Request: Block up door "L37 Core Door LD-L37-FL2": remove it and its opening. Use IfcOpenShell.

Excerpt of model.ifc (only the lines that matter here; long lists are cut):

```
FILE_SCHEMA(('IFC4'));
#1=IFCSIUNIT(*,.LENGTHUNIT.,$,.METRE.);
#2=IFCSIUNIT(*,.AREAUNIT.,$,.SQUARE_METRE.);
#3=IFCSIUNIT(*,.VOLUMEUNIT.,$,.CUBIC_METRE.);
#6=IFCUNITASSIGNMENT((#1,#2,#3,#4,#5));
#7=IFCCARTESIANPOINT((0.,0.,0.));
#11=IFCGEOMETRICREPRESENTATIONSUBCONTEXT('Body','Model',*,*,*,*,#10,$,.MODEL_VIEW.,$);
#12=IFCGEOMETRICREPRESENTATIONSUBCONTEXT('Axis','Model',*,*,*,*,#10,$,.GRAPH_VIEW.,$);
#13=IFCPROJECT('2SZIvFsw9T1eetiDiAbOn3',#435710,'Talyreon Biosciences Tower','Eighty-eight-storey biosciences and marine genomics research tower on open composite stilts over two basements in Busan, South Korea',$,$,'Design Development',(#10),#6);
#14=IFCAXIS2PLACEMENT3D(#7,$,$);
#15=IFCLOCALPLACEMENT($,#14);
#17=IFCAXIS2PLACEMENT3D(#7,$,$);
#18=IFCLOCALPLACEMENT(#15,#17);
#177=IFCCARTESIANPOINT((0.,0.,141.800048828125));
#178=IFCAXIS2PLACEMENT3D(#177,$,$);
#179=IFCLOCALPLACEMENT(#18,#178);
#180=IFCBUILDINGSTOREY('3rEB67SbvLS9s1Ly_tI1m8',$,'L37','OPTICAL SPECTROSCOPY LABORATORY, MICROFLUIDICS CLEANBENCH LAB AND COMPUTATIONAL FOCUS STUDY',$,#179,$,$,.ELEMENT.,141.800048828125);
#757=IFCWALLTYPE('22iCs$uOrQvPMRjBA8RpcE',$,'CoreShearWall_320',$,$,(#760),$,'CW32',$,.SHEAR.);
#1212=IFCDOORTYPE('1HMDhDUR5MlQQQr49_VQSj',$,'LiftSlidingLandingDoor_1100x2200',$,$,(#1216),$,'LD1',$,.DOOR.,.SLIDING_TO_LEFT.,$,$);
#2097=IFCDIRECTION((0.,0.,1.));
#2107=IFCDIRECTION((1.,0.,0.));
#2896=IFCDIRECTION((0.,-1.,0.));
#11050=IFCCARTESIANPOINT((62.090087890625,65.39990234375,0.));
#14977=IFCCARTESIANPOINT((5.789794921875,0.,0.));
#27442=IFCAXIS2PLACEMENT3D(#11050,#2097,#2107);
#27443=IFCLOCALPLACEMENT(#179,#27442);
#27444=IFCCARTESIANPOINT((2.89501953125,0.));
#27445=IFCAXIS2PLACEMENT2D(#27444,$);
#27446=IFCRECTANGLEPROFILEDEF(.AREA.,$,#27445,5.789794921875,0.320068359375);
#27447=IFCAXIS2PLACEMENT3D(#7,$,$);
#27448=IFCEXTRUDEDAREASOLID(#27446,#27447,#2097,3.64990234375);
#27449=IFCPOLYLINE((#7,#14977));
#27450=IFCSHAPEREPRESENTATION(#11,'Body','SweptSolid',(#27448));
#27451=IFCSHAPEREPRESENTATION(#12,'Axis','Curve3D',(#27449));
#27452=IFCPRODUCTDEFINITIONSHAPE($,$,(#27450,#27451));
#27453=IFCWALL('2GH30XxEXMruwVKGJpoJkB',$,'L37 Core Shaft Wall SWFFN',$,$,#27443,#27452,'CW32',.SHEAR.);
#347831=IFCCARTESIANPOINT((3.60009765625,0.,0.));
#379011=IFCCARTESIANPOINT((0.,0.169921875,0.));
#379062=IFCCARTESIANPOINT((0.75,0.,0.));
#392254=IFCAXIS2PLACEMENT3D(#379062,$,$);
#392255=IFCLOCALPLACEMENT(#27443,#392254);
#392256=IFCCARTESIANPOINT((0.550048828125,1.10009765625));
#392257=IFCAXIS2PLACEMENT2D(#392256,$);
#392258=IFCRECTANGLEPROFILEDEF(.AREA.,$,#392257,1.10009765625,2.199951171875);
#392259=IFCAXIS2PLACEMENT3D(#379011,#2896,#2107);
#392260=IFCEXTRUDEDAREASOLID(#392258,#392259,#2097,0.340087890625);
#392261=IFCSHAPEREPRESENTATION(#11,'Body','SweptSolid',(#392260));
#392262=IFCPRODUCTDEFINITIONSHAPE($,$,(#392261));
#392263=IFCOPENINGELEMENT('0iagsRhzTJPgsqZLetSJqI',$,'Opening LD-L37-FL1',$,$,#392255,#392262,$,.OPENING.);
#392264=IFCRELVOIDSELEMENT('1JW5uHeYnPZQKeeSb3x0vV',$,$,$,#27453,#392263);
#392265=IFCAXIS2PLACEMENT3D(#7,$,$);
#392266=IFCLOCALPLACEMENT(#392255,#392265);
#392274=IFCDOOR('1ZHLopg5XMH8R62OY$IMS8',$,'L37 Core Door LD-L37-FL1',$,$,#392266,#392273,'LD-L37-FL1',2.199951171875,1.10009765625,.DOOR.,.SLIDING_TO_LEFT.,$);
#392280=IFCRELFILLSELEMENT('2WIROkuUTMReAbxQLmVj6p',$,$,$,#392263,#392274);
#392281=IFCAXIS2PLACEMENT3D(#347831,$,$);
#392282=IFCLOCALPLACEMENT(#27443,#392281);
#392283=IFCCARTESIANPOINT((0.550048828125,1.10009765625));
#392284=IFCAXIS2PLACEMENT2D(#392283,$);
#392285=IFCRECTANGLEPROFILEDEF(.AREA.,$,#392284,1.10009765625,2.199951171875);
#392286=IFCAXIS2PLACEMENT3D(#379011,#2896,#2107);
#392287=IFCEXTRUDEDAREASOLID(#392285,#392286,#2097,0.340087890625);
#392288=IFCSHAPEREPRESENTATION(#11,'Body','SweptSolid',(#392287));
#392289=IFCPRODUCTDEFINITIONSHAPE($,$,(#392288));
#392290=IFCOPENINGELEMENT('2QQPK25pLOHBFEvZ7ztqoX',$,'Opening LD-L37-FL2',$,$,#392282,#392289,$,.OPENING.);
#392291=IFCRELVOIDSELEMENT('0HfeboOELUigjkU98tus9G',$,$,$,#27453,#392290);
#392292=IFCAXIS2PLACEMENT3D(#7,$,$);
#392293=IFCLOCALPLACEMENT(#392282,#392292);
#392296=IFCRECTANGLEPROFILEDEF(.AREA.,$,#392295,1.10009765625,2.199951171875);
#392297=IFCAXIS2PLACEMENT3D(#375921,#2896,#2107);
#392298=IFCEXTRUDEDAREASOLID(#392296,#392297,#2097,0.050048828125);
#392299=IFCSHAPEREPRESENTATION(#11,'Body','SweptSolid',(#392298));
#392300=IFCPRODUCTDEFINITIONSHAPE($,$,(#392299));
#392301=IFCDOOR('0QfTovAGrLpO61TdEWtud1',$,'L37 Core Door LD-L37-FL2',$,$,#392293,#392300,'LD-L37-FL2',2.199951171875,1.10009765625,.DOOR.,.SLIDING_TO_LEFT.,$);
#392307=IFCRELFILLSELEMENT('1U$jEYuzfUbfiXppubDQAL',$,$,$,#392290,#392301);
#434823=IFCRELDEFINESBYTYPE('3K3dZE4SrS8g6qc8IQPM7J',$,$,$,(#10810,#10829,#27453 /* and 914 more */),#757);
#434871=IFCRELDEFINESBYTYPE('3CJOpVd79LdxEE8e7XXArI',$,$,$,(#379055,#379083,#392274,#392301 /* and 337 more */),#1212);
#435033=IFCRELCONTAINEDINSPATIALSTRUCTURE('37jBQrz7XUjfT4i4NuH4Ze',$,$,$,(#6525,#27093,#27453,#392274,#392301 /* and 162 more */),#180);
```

```python
import ifcopenshell
import ifcopenshell.api.feature
import ifcopenshell.api.root
import ifcopenshell.geom
import ifcopenshell.util.shape

model = ifcopenshell.open("model.ifc")
settings = ifcopenshell.geom.settings()


def volume(element):
    """Net volume in cubic metres, openings subtracted."""
    shape = ifcopenshell.geom.create_shape(settings, element)
    return ifcopenshell.util.shape.get_volume(shape.geometry)


door = model.by_guid("0QfTovAGrLpO61TdEWtud1")
opening = door.FillsVoids[0].RelatingOpeningElement
wall = opening.VoidsElements[0].RelatingBuildingElement
before = volume(wall)

ifcopenshell.api.root.remove_product(model, product=door)
ifcopenshell.api.feature.remove_feature(model, feature=opening)

after = volume(wall)

print(f"wall volume {before:.3f} -> {after:.3f} m3")

model.write("model_edited.ifc")
```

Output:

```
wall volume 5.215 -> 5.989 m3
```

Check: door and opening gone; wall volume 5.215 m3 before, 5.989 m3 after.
